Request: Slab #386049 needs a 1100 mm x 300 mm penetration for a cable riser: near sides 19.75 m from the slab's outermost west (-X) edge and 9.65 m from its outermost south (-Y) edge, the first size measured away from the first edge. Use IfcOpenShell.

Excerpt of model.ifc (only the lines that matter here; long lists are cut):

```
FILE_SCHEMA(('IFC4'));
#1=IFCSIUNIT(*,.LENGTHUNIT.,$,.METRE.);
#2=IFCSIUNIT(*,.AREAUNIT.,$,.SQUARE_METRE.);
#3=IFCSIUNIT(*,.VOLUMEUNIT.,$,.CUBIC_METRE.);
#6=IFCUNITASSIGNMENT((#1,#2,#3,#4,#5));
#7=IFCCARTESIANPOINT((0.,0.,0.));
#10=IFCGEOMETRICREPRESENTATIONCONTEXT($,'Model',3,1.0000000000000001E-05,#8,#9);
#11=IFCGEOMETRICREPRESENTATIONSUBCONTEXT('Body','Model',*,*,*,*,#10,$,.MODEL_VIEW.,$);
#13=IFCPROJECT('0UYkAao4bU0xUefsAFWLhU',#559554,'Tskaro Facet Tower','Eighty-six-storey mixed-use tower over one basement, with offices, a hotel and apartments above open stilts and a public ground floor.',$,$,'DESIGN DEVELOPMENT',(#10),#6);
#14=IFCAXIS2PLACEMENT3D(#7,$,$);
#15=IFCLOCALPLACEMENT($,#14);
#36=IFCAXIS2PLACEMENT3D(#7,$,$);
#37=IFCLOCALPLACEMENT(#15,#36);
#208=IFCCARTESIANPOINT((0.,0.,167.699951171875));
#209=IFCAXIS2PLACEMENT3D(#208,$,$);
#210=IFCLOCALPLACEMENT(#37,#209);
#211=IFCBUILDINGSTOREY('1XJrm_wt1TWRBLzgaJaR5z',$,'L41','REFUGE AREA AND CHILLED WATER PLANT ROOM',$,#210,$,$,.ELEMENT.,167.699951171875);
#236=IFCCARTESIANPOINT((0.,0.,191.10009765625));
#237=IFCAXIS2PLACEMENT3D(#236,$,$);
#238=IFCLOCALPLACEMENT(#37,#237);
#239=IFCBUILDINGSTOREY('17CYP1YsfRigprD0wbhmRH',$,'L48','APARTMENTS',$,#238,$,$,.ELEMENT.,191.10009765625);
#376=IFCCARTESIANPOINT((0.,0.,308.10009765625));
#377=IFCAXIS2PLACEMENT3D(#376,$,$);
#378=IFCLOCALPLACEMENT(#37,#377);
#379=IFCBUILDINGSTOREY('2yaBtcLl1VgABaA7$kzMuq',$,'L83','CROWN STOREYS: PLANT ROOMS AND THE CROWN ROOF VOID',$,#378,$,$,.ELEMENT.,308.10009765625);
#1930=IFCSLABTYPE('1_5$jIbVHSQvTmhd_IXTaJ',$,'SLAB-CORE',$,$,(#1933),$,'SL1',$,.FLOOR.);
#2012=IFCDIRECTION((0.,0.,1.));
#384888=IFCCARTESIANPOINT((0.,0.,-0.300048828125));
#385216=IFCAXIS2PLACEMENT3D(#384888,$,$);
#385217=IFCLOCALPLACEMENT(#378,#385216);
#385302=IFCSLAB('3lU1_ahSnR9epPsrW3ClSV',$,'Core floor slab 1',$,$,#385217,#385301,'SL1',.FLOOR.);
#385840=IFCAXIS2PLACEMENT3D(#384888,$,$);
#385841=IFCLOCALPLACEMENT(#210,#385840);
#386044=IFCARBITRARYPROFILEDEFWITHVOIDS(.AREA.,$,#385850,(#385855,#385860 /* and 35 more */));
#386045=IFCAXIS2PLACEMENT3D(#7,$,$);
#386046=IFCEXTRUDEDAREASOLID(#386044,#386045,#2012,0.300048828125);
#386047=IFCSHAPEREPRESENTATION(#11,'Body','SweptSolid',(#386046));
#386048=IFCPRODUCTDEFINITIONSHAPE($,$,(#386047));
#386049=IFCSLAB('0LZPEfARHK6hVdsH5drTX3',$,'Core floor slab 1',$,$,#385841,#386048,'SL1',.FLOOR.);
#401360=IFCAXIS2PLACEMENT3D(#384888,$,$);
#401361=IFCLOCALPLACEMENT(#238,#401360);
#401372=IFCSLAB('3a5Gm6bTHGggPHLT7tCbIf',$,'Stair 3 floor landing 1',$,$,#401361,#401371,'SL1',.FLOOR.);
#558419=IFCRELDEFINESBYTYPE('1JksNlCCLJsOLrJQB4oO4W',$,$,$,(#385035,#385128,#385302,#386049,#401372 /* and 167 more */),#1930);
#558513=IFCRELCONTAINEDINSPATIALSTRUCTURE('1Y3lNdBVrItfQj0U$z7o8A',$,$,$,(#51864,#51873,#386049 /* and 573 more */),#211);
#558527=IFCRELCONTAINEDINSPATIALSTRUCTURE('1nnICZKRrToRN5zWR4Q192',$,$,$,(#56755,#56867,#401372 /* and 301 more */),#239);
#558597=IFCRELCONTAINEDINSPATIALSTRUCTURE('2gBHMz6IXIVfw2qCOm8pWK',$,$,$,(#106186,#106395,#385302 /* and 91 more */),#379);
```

```python
import numpy as np
import ifcopenshell
import ifcopenshell.api.feature
import ifcopenshell.api.geometry
import ifcopenshell.api.root
import ifcopenshell.geom
import ifcopenshell.util.placement
import ifcopenshell.util.representation
import ifcopenshell.util.shape
import ifcopenshell.util.unit

model = ifcopenshell.open("model.ifc")
unit_scale = ifcopenshell.util.unit.calculate_unit_scale(model)
settings = ifcopenshell.geom.settings()


def volume(element):
    """Net volume in cubic metres, openings subtracted."""
    shape = ifcopenshell.geom.create_shape(settings, element)
    return ifcopenshell.util.shape.get_volume(shape.geometry)


slab = model.by_guid("0LZPEfARHK6hVdsH5drTX3")
before = volume(slab)

# Extent in the slab's own axes, in metres. The edges named are its -X and -Y sides.
slab_shape = ifcopenshell.geom.create_shape(settings, slab)
vertices = ifcopenshell.util.shape.get_vertices(slab_shape.geometry)
x_min, y_min, bottom = vertices.min(axis=0)
top = vertices[:, 2].max()

opening = ifcopenshell.api.root.create_entity(model, ifc_class="IfcOpeningElement", name="Cable riser opening", predefined_type="OPENING")
context = ifcopenshell.util.representation.get_context(model, "Model", "Body", "MODEL_VIEW")
width, depth = 1.1, 0.3
outline = [(0.0, 0.0), (width, 0.0), (width, depth), (0.0, depth), (0.0, 0.0)]
# Overshoot both faces by 50 mm so the cut is clean.
shape = ifcopenshell.api.geometry.add_slab_representation(
    model, context=context, depth=top - bottom + 0.1, polyline=outline
)
ifcopenshell.api.geometry.assign_representation(model, product=opening, representation=shape)

matrix = ifcopenshell.util.placement.get_local_placement(slab.ObjectPlacement)
matrix[:, 3] = matrix @ np.append(np.array([x_min + 19.75, y_min + 9.65, bottom - 0.05]) / unit_scale, 1.0)
ifcopenshell.api.geometry.edit_object_placement(model, product=opening, matrix=matrix, is_si=False)
ifcopenshell.api.feature.add_feature(model, feature=opening, element=slab)

after = volume(slab)

print(f"slab volume {before:.3f} -> {after:.3f} m3")

model.write("model_rev.ifc")
```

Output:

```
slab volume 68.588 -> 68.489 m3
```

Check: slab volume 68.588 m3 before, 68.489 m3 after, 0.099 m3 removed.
